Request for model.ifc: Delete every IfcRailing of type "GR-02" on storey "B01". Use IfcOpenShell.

First a look at what the model holds.

```python
import ifcopenshell
import ifcopenshell.util.element

model = ifcopenshell.open("model.ifc")
print(model.schema)
storey = next(s for s in model.by_type("IfcBuildingStorey") if s.Name == "B01")
railings = [e for e in ifcopenshell.util.element.get_decomposition(storey) if e.is_a("IfcRailing")]
seen = {}
for e in railings:
    element_type = ifcopenshell.util.element.get_type(e)
    name = element_type.Name if element_type not in (None, e) else None
    seen[name] = seen.get(name, 0) + 1
for name, count in sorted(seen.items(), key=str):
    print(count, "x", name)
```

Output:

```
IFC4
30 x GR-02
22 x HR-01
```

```python
import ifcopenshell
import ifcopenshell.api.root
import ifcopenshell.util.element

model = ifcopenshell.open("model.ifc")

storey = next(s for s in model.by_type("IfcBuildingStorey") if s.Name == "B01")
railings = [e for e in ifcopenshell.util.element.get_decomposition(storey) if e.is_a("IfcRailing")]
targets = [e for e in railings if (t := ifcopenshell.util.element.get_type(e)) not in (None, e) and t.Name == "GR-02"]

for e in targets:
    ifcopenshell.api.root.remove_product(model, product=e)
print(len(targets), "removed")

model.write("model-out.ifc")
```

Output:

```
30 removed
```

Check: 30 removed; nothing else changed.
